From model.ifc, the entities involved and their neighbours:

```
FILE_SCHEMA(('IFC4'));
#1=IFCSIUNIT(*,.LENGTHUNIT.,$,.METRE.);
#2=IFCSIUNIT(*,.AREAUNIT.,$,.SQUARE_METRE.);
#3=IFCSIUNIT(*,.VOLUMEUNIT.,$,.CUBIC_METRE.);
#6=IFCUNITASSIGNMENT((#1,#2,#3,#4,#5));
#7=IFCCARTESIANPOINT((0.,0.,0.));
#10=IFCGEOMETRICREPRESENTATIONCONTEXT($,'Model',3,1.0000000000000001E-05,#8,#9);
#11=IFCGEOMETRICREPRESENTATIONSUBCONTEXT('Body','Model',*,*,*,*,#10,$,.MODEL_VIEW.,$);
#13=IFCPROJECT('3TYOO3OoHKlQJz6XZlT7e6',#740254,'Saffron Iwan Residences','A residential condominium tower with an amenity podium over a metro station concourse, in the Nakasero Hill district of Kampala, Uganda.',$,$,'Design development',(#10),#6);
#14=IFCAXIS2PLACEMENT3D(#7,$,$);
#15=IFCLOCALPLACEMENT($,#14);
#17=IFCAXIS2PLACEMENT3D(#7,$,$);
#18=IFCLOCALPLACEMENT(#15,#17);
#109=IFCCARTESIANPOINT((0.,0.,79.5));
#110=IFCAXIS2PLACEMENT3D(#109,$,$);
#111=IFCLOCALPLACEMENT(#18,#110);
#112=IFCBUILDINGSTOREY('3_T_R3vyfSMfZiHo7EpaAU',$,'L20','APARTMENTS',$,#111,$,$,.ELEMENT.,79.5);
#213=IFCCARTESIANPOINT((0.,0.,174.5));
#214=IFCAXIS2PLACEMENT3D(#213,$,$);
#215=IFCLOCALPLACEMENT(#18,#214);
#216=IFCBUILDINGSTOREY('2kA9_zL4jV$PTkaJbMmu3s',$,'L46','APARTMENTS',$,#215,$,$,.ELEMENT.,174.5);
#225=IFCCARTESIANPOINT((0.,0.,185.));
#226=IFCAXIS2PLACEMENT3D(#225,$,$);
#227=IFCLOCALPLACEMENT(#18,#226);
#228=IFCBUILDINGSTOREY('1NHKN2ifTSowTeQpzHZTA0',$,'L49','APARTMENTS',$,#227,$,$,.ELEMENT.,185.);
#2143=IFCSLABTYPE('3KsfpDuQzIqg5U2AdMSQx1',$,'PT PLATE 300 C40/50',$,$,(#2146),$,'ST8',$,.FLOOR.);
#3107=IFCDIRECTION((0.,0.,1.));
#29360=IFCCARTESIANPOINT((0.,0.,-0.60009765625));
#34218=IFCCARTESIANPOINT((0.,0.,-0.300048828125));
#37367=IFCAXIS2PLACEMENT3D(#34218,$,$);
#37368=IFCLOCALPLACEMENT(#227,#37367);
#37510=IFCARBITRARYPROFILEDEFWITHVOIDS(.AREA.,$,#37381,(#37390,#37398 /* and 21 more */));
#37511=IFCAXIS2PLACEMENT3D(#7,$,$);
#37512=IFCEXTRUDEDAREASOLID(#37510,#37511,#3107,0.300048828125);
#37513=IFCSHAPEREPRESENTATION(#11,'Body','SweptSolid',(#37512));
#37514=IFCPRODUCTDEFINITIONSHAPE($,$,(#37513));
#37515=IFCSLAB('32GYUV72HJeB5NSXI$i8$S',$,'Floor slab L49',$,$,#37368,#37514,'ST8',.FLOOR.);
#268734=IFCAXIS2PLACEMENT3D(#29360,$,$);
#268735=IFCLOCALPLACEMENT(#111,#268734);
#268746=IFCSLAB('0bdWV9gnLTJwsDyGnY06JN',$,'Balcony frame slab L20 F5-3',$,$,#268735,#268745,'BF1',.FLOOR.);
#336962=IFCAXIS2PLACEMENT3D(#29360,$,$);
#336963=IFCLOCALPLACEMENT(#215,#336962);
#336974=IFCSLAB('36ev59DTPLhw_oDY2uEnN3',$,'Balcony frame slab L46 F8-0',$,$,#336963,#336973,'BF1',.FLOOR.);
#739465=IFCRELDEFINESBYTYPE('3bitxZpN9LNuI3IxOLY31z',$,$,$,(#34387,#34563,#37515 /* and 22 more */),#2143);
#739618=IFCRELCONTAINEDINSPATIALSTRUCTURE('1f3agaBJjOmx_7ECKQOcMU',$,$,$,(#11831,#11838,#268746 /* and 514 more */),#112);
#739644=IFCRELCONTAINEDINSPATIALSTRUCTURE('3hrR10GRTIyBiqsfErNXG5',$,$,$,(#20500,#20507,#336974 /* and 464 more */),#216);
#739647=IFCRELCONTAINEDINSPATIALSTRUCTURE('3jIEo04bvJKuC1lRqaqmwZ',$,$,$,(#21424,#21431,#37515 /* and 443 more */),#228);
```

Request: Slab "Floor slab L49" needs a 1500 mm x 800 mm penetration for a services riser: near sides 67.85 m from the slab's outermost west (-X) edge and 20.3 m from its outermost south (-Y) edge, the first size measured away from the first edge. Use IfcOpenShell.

```python
import numpy as np
import ifcopenshell
import ifcopenshell.api.feature
import ifcopenshell.api.geometry
import ifcopenshell.api.root
import ifcopenshell.geom
import ifcopenshell.util.placement
import ifcopenshell.util.representation
import ifcopenshell.util.shape
import ifcopenshell.util.unit

model = ifcopenshell.open("model.ifc")
unit_scale = ifcopenshell.util.unit.calculate_unit_scale(model)
settings = ifcopenshell.geom.settings()


def volume(element):
    """Net volume in cubic metres, openings subtracted."""
    shape = ifcopenshell.geom.create_shape(settings, element)
    return ifcopenshell.util.shape.get_volume(shape.geometry)


slab = model.by_guid("32GYUV72HJeB5NSXI$i8$S")
before = volume(slab)

# Extent in the slab's own axes, in metres. The edges named are its -X and -Y sides.
slab_shape = ifcopenshell.geom.create_shape(settings, slab)
vertices = ifcopenshell.util.shape.get_vertices(slab_shape.geometry)
x_min, y_min, bottom = vertices.min(axis=0)
top = vertices[:, 2].max()

opening = ifcopenshell.api.root.create_entity(model, ifc_class="IfcOpeningElement", name="Services riser opening", predefined_type="OPENING")
context = ifcopenshell.util.representation.get_context(model, "Model", "Body", "MODEL_VIEW")
width, depth = 1.5, 0.8
outline = [(0.0, 0.0), (width, 0.0), (width, depth), (0.0, depth), (0.0, 0.0)]
# Overshoot both faces by 50 mm so the cut is clean.
shape = ifcopenshell.api.geometry.add_slab_representation(
    model, context=context, depth=top - bottom + 0.1, polyline=outline
)
ifcopenshell.api.geometry.assign_representation(model, product=opening, representation=shape)

matrix = ifcopenshell.util.placement.get_local_placement(slab.ObjectPlacement)
matrix[:, 3] = matrix @ np.append(np.array([x_min + 67.85, y_min + 20.3, bottom - 0.05]) / unit_scale, 1.0)
ifcopenshell.api.geometry.edit_object_placement(model, product=opening, matrix=matrix, is_si=False)
ifcopenshell.api.feature.add_feature(model, feature=opening, element=slab)

after = volume(slab)

print(f"slab volume {before:.3f} -> {after:.3f} m3")

model.write("model_edited.ifc")
```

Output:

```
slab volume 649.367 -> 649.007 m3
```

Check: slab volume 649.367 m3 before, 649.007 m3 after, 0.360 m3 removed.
